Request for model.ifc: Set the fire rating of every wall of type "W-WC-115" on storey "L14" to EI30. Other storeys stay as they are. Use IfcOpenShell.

First a look at what the model holds.

```python
import ifcopenshell
import ifcopenshell.util.element

model = ifcopenshell.open("model.ifc")
print(model.schema)
storey = next(s for s in model.by_type("IfcBuildingStorey") if s.Name == "L14")
walls = [e for e in ifcopenshell.util.element.get_decomposition(storey) if e.is_a("IfcWall")]
seen = {}
for e in walls:
    element_type = ifcopenshell.util.element.get_type(e)
    key = (element_type.Name if element_type != e and element_type else None, ifcopenshell.util.element.get_pset(e, "Pset_WallCommon", "FireRating"))
    seen[key] = seen.get(key, 0) + 1
for (name, value), count in sorted(seen.items(), key=str):
    print(count, "x", name, "|", value)
```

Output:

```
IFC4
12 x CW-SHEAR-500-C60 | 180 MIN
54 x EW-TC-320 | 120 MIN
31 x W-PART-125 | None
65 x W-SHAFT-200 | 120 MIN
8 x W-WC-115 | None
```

```python
import ifcopenshell
import ifcopenshell.api.pset
import ifcopenshell.util.element

model = ifcopenshell.open("model.ifc")

storey = next(s for s in model.by_type("IfcBuildingStorey") if s.Name == "L14")
walls = [e for e in ifcopenshell.util.element.get_decomposition(storey) if e.is_a("IfcWall")]

count = 0
for e in walls:
    element_type = ifcopenshell.util.element.get_type(e)
    if element_type in (None, e) or element_type.Name != "W-WC-115":
        continue
    found = ifcopenshell.util.element.get_pset(e, "Pset_WallCommon", should_inherit=False)
    if found:
        pset = model.by_id(found["id"])
        if len(ifcopenshell.util.element.get_elements_by_pset(pset)) > 1:
            pset = ifcopenshell.api.pset.unshare_pset(model, products=[e], pset=pset)[0]
    else:
        pset = ifcopenshell.api.pset.add_pset(model, product=e, name="Pset_WallCommon")
    ifcopenshell.api.pset.edit_pset(model, pset=pset, properties={"FireRating": "EI30"})
    count += 1

print(count, "walls updated")

model.write("model_rev.ifc")
```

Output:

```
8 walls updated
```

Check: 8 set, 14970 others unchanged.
